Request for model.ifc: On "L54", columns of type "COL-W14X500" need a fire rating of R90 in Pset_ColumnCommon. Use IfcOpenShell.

First a look at what the model holds.

```python
import ifcopenshell
import ifcopenshell.util.element

model = ifcopenshell.open("model.ifc")
print(model.schema)
storey = next(s for s in model.by_type("IfcBuildingStorey") if s.Name == "L54")
columns = [e for e in ifcopenshell.util.element.get_decomposition(storey) if e.is_a("IfcColumn")]
seen = {}
for e in columns:
    element_type = ifcopenshell.util.element.get_type(e)
    key = (element_type.Name if element_type != e and element_type else None, ifcopenshell.util.element.get_pset(e, "Pset_ColumnCommon", "FireRating"))
    seen[key] = seen.get(key, 0) + 1
for (name, value), count in sorted(seen.items(), key=str):
    print(count, "x", name, "|", value)
```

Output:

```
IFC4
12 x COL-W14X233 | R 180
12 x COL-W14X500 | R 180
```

```python
import ifcopenshell
import ifcopenshell.api.pset
import ifcopenshell.util.element

model = ifcopenshell.open("model.ifc")

storey = next(s for s in model.by_type("IfcBuildingStorey") if s.Name == "L54")
columns = [e for e in ifcopenshell.util.element.get_decomposition(storey) if e.is_a("IfcColumn")]

count = 0
for e in columns:
    element_type = ifcopenshell.util.element.get_type(e)
    if element_type in (None, e) or element_type.Name != "COL-W14X500":
        continue
    found = ifcopenshell.util.element.get_pset(e, "Pset_ColumnCommon", should_inherit=False)
    if found:
        pset = model.by_id(found["id"])
        if len(ifcopenshell.util.element.get_elements_by_pset(pset)) > 1:
            pset = ifcopenshell.api.pset.unshare_pset(model, products=[e], pset=pset)[0]
    else:
        pset = ifcopenshell.api.pset.add_pset(model, product=e, name="Pset_ColumnCommon")
    ifcopenshell.api.pset.edit_pset(model, pset=pset, properties={"FireRating": "R90"})
    count += 1

print(count, "columns updated")

model.write("model_v2.ifc")
```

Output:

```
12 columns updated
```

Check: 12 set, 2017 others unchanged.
